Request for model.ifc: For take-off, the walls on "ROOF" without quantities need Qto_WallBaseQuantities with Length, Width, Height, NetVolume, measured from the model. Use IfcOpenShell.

First a look at what the model holds.

```python
import ifcopenshell
import ifcopenshell.util.element
import ifcopenshell.util.unit

model = ifcopenshell.open("model.ifc")
print(model.schema)
for unit_type in ("LENGTHUNIT", "AREAUNIT", "VOLUMEUNIT"):
    print(unit_type, ifcopenshell.util.unit.calculate_unit_scale(model, unit_type))
storey = next(s for s in model.by_type("IfcBuildingStorey") if s.Name == "ROOF")
walls = [e for e in ifcopenshell.util.element.get_decomposition(storey) if e.is_a("IfcWall")]
for e in sorted(walls, key=lambda e: e.id()):
    print(e.id(), e.is_a(), e.Name, list(ifcopenshell.util.element.get_psets(e, qtos_only=True)), sep=" | ")
```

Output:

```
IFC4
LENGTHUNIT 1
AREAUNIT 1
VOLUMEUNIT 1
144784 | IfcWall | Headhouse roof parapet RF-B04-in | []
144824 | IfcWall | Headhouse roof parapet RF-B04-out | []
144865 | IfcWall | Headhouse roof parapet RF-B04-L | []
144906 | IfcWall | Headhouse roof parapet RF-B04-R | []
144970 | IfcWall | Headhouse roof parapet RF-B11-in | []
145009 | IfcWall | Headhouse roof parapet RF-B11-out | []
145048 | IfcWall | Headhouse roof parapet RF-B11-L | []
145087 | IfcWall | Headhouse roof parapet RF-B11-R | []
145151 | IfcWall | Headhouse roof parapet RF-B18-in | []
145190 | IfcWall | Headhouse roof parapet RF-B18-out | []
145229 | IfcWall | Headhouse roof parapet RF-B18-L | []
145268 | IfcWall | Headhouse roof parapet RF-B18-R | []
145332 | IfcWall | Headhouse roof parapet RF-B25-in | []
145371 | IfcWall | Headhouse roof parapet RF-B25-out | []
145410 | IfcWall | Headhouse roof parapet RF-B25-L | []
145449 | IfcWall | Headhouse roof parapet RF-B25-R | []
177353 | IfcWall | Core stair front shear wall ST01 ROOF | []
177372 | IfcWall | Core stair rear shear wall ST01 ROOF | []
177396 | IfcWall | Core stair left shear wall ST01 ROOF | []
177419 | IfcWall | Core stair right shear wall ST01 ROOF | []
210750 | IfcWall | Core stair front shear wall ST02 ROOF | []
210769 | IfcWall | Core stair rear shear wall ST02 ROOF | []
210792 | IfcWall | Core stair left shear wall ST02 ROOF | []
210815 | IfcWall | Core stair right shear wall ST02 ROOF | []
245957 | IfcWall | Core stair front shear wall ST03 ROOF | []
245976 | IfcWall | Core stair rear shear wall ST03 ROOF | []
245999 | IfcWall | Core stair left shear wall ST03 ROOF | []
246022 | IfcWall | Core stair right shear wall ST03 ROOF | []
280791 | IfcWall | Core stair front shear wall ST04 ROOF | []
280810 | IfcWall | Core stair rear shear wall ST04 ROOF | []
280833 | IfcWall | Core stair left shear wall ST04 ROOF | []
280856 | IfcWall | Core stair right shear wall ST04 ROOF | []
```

```python
import ifcopenshell
import ifcopenshell.api.pset
import ifcopenshell.geom
import ifcopenshell.util.element
import ifcopenshell.util.shape
import ifcopenshell.util.unit

model = ifcopenshell.open("model.ifc")
unit_scale = ifcopenshell.util.unit.calculate_unit_scale(model)
volume_scale = ifcopenshell.util.unit.calculate_unit_scale(model, "VOLUMEUNIT")
settings = ifcopenshell.geom.settings()

storey = next(s for s in model.by_type("IfcBuildingStorey") if s.Name == "ROOF")
walls = [e for e in ifcopenshell.util.element.get_decomposition(storey) if e.is_a("IfcWall")]

for e in sorted(walls, key=lambda e: e.id()):
    if ifcopenshell.util.element.get_psets(e, qtos_only=True, should_inherit=False):
        continue
    # Geometry comes back in metres, in the element's own axes.
    shape = ifcopenshell.geom.create_shape(settings, e)
    values = {
        "Length": ifcopenshell.util.shape.get_x(shape.geometry) / unit_scale,
        "Width": ifcopenshell.util.shape.get_y(shape.geometry) / unit_scale,
        "Height": ifcopenshell.util.shape.get_z(shape.geometry) / unit_scale,
        "NetVolume": ifcopenshell.util.shape.get_volume(shape.geometry) / volume_scale,
    }
    qto = ifcopenshell.api.pset.add_qto(model, product=e, name="Qto_WallBaseQuantities")
    ifcopenshell.api.pset.edit_qto(model, qto=qto, properties=values)
    print(e.id(), {k: round(v, 3) for k, v in values.items()})

model.write("model_updated.ifc")
```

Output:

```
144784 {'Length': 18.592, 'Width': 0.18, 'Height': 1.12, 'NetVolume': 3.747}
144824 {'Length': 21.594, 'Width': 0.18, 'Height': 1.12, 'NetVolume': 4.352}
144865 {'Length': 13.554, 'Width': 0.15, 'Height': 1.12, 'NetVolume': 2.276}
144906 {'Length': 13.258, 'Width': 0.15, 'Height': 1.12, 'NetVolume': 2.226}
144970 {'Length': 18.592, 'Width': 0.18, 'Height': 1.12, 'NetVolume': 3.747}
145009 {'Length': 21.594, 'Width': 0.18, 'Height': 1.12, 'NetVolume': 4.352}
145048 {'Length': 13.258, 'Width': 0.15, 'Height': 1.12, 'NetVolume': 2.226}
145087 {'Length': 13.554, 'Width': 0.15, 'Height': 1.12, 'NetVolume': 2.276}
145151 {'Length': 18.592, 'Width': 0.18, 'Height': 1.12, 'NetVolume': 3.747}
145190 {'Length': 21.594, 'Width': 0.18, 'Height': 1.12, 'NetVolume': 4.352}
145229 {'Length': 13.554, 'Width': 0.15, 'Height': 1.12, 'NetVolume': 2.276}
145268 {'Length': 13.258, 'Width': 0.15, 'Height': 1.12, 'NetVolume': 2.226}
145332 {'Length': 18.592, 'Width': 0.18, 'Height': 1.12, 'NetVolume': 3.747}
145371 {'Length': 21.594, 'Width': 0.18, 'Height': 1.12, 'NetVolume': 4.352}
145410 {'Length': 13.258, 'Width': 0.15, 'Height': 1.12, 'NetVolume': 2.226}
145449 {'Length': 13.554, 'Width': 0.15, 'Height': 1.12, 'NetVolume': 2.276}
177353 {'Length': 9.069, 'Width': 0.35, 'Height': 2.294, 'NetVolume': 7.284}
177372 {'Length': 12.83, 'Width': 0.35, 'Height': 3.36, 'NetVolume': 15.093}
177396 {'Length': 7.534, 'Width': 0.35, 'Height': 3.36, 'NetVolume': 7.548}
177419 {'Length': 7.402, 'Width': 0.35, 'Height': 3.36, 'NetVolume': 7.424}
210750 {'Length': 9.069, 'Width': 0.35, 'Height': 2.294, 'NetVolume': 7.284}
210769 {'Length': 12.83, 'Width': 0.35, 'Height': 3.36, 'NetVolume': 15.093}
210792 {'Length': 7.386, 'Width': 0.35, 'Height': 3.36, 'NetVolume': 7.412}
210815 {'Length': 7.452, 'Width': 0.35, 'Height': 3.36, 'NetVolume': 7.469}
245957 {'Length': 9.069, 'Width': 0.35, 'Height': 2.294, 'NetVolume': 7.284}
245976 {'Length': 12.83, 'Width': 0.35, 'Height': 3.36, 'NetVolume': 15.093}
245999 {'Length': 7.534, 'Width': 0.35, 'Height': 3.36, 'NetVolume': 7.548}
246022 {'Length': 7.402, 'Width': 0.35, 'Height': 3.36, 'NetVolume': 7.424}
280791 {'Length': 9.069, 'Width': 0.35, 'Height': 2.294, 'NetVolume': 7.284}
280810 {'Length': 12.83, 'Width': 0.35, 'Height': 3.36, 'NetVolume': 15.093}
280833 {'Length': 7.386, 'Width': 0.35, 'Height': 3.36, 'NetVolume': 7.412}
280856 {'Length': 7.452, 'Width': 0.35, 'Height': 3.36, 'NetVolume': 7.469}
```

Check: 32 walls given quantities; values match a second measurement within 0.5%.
